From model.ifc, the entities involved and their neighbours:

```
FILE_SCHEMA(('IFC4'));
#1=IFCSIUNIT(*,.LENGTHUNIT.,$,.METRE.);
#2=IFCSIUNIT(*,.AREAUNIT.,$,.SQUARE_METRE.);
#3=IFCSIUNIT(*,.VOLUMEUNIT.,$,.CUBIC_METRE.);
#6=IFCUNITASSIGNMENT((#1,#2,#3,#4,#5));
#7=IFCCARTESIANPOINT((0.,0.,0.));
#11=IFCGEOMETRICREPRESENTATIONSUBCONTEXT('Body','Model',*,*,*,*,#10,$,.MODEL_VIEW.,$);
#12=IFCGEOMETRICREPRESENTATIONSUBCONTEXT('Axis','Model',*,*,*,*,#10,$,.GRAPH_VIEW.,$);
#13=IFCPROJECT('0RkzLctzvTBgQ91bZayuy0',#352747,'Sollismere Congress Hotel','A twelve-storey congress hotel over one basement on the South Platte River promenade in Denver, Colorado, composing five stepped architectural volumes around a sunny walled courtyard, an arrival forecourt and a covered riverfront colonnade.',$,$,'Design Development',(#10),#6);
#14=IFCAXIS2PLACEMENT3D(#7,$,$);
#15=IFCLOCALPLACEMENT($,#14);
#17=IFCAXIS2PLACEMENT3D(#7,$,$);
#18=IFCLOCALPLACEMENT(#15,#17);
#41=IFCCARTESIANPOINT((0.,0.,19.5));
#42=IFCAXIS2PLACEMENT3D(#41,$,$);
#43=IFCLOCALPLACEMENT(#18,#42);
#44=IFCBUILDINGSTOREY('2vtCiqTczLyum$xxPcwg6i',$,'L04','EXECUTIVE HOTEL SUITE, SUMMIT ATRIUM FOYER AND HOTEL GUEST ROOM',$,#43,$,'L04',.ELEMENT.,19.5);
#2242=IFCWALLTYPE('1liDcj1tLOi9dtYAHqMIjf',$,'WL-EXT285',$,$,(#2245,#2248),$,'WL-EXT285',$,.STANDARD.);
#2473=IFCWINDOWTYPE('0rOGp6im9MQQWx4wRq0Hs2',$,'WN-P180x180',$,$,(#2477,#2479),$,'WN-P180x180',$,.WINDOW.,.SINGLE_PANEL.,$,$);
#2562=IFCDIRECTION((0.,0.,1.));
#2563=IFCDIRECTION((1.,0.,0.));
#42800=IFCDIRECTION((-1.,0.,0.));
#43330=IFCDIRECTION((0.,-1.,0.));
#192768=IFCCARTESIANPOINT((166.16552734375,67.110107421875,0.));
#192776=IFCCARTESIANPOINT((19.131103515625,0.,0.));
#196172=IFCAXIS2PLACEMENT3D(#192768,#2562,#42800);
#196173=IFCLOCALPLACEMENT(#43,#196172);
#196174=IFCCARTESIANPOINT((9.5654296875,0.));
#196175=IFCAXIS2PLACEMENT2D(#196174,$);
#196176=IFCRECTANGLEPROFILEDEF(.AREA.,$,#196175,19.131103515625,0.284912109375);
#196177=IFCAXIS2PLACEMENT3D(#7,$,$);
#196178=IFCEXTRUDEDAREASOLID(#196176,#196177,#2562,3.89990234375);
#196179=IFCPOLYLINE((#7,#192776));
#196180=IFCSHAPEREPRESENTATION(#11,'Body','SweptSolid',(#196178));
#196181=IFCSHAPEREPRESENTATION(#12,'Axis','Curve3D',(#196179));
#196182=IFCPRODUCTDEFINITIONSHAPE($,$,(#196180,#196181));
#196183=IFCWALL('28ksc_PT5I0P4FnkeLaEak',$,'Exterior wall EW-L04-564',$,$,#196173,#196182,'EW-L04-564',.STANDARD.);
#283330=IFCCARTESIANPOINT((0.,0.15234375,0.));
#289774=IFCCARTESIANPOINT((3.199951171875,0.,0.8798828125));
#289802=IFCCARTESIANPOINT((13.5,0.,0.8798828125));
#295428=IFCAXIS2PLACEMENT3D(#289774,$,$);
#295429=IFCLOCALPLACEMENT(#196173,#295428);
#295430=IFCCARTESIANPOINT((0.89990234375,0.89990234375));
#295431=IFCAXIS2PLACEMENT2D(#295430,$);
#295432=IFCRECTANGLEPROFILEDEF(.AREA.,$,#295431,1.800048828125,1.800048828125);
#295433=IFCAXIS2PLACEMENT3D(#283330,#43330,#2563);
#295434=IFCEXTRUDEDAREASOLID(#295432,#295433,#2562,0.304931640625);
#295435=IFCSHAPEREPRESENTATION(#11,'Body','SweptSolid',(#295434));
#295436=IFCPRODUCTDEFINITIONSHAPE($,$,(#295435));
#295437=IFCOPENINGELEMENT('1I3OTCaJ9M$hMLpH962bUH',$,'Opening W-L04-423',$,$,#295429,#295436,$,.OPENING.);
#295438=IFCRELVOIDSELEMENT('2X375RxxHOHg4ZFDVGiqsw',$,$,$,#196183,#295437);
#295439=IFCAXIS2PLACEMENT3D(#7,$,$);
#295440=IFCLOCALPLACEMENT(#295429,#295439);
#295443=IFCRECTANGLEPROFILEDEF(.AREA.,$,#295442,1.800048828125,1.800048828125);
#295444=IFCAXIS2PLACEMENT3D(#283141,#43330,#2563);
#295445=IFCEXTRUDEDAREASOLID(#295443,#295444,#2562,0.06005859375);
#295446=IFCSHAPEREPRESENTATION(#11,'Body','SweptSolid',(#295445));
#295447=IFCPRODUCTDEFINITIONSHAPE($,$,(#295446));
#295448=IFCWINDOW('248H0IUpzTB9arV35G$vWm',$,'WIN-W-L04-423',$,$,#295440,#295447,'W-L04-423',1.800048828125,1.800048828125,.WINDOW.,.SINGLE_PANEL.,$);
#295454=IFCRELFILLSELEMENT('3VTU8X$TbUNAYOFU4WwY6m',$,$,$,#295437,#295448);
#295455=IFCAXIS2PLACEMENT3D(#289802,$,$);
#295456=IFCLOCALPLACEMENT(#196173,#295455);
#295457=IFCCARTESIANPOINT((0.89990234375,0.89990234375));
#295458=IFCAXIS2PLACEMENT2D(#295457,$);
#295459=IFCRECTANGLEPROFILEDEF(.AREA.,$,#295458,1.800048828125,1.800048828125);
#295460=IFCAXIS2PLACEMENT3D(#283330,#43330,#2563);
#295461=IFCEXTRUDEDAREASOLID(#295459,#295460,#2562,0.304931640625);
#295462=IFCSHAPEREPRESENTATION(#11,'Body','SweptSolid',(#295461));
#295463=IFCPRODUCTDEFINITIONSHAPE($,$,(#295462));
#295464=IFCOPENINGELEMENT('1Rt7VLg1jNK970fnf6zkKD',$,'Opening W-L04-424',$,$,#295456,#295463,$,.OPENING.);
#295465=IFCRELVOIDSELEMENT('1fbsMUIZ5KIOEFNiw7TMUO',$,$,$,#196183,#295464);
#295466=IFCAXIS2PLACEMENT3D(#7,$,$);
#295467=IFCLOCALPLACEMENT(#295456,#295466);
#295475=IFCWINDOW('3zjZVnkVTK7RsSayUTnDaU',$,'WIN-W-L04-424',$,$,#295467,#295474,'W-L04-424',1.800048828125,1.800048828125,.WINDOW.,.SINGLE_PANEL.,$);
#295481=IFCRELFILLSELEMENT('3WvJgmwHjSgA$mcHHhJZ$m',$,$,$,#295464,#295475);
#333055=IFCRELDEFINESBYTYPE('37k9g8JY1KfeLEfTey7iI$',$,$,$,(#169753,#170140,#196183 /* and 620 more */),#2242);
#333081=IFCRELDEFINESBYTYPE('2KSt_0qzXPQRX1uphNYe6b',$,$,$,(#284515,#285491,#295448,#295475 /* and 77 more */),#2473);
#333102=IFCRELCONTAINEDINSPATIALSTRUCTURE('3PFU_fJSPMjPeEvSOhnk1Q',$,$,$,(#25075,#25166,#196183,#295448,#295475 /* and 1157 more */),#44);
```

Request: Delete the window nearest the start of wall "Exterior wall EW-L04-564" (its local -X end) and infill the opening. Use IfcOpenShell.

```python
import ifcopenshell
import ifcopenshell.api.feature
import ifcopenshell.api.root
import ifcopenshell.geom
import ifcopenshell.util.shape

model = ifcopenshell.open("model.ifc")
settings = ifcopenshell.geom.settings()


def volume(element):
    """Net volume in cubic metres, openings subtracted."""
    shape = ifcopenshell.geom.create_shape(settings, element)
    return ifcopenshell.util.shape.get_volume(shape.geometry)


window = model.by_guid("248H0IUpzTB9arV35G$vWm")
opening = window.FillsVoids[0].RelatingOpeningElement
wall = opening.VoidsElements[0].RelatingBuildingElement
before = volume(wall)

ifcopenshell.api.root.remove_product(model, product=window)
ifcopenshell.api.feature.remove_feature(model, feature=opening)

after = volume(wall)

print(f"wall volume {before:.3f} -> {after:.3f} m3")

model.write("model_edited.ifc")
```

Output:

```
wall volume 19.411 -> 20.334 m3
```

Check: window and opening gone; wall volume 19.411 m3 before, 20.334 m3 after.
